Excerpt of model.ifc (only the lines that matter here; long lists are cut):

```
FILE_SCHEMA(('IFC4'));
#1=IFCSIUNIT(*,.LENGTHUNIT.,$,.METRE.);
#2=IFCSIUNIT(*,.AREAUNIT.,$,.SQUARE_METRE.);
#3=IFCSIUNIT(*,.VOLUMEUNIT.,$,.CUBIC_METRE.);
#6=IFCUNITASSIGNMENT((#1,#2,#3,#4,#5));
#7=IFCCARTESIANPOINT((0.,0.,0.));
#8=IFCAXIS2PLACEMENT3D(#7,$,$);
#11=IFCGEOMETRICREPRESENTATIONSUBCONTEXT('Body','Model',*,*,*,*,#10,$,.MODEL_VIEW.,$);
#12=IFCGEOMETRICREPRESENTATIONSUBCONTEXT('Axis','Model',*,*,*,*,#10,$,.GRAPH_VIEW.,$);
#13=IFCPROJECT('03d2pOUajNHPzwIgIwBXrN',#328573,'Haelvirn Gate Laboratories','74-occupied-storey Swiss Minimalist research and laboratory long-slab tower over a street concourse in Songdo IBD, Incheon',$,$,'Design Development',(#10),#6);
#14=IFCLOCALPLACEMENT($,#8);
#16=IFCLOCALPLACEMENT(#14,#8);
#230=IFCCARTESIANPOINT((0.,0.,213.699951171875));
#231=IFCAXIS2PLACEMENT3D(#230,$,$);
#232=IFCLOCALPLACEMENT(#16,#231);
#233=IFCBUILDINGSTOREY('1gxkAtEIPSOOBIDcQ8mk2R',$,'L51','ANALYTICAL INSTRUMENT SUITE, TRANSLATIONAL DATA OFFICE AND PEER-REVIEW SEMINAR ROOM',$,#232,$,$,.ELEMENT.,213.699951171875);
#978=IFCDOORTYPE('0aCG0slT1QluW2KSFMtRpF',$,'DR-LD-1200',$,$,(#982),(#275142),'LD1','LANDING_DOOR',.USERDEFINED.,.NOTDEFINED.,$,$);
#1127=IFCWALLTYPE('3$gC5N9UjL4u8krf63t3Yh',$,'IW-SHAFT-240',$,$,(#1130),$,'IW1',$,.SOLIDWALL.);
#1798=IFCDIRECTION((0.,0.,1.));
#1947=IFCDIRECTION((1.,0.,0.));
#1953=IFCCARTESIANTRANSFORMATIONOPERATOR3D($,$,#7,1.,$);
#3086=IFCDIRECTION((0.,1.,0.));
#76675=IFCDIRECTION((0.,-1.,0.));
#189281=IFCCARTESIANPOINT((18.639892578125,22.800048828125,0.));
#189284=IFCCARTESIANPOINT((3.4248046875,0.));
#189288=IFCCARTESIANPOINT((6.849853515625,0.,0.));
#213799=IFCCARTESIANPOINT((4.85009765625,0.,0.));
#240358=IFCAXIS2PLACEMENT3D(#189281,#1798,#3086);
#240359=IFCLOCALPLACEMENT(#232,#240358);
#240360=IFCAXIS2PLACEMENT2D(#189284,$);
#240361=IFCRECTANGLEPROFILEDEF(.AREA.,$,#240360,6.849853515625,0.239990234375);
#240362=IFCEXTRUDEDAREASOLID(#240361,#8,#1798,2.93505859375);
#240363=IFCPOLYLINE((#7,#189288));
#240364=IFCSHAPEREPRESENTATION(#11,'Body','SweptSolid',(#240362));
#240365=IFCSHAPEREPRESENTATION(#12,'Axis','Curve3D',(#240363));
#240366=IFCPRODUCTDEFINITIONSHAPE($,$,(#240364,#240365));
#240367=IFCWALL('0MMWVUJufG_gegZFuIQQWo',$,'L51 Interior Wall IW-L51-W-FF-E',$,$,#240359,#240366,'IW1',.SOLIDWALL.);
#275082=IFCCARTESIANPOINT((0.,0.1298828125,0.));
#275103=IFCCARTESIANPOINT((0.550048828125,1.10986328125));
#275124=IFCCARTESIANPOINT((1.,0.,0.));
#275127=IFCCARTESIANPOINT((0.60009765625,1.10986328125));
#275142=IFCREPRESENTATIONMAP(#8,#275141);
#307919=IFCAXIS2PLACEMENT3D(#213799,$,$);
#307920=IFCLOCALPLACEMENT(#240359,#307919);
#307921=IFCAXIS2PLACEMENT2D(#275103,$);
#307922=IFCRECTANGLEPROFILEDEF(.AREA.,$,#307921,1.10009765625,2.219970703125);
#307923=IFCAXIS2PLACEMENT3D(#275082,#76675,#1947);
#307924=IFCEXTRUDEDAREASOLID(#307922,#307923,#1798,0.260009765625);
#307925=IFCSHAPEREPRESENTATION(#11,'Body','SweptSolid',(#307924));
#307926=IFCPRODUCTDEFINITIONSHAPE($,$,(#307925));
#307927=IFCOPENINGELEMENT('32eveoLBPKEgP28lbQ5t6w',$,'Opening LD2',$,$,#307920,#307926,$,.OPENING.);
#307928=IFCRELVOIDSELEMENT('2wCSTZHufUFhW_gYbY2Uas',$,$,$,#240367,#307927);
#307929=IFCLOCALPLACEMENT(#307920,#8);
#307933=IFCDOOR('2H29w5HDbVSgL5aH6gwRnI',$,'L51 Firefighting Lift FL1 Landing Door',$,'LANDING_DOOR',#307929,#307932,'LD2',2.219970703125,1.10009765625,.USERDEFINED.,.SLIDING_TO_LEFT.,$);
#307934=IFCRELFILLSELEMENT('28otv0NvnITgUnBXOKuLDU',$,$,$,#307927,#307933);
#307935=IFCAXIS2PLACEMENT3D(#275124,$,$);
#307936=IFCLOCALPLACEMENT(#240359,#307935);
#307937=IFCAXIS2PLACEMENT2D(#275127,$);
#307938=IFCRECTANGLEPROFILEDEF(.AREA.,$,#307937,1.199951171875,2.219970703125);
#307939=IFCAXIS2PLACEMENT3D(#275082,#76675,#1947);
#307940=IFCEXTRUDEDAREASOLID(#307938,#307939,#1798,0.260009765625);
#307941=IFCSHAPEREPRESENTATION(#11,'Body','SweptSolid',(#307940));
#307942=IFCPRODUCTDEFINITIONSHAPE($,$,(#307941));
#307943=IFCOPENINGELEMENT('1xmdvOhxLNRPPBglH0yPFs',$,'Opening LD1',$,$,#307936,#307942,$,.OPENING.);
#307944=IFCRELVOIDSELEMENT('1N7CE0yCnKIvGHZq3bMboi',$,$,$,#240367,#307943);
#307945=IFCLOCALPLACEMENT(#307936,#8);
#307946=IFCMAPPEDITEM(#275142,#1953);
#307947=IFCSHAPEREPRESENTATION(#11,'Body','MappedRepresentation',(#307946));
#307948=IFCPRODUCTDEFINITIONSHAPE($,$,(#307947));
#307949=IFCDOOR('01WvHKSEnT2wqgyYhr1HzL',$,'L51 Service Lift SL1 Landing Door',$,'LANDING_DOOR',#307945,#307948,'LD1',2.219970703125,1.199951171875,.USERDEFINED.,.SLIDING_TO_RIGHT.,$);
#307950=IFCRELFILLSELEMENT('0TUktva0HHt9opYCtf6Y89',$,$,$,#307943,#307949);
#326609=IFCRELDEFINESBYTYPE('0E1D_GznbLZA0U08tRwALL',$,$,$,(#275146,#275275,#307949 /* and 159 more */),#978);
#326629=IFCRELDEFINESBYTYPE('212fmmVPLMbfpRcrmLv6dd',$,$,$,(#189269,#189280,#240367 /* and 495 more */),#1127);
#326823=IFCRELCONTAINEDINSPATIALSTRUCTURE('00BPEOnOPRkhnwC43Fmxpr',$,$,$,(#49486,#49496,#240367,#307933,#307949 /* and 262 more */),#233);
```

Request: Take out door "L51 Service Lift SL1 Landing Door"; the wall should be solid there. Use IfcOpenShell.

```python
import ifcopenshell
import ifcopenshell.api.feature
import ifcopenshell.api.root
import ifcopenshell.geom
import ifcopenshell.util.shape

model = ifcopenshell.open("model.ifc")
settings = ifcopenshell.geom.settings()


def volume(element):
    """Net volume in cubic metres, openings subtracted."""
    shape = ifcopenshell.geom.create_shape(settings, element)
    return ifcopenshell.util.shape.get_volume(shape.geometry)


door = model.by_guid("01WvHKSEnT2wqgyYhr1HzL")
opening = door.FillsVoids[0].RelatingOpeningElement
wall = opening.VoidsElements[0].RelatingBuildingElement
before = volume(wall)

ifcopenshell.api.root.remove_product(model, product=door)
ifcopenshell.api.feature.remove_feature(model, feature=opening)

after = volume(wall)

print(f"wall volume {before:.3f} -> {after:.3f} m3")

model.write("model_updated.ifc")
```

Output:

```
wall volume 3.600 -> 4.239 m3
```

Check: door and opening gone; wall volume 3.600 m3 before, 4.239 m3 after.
